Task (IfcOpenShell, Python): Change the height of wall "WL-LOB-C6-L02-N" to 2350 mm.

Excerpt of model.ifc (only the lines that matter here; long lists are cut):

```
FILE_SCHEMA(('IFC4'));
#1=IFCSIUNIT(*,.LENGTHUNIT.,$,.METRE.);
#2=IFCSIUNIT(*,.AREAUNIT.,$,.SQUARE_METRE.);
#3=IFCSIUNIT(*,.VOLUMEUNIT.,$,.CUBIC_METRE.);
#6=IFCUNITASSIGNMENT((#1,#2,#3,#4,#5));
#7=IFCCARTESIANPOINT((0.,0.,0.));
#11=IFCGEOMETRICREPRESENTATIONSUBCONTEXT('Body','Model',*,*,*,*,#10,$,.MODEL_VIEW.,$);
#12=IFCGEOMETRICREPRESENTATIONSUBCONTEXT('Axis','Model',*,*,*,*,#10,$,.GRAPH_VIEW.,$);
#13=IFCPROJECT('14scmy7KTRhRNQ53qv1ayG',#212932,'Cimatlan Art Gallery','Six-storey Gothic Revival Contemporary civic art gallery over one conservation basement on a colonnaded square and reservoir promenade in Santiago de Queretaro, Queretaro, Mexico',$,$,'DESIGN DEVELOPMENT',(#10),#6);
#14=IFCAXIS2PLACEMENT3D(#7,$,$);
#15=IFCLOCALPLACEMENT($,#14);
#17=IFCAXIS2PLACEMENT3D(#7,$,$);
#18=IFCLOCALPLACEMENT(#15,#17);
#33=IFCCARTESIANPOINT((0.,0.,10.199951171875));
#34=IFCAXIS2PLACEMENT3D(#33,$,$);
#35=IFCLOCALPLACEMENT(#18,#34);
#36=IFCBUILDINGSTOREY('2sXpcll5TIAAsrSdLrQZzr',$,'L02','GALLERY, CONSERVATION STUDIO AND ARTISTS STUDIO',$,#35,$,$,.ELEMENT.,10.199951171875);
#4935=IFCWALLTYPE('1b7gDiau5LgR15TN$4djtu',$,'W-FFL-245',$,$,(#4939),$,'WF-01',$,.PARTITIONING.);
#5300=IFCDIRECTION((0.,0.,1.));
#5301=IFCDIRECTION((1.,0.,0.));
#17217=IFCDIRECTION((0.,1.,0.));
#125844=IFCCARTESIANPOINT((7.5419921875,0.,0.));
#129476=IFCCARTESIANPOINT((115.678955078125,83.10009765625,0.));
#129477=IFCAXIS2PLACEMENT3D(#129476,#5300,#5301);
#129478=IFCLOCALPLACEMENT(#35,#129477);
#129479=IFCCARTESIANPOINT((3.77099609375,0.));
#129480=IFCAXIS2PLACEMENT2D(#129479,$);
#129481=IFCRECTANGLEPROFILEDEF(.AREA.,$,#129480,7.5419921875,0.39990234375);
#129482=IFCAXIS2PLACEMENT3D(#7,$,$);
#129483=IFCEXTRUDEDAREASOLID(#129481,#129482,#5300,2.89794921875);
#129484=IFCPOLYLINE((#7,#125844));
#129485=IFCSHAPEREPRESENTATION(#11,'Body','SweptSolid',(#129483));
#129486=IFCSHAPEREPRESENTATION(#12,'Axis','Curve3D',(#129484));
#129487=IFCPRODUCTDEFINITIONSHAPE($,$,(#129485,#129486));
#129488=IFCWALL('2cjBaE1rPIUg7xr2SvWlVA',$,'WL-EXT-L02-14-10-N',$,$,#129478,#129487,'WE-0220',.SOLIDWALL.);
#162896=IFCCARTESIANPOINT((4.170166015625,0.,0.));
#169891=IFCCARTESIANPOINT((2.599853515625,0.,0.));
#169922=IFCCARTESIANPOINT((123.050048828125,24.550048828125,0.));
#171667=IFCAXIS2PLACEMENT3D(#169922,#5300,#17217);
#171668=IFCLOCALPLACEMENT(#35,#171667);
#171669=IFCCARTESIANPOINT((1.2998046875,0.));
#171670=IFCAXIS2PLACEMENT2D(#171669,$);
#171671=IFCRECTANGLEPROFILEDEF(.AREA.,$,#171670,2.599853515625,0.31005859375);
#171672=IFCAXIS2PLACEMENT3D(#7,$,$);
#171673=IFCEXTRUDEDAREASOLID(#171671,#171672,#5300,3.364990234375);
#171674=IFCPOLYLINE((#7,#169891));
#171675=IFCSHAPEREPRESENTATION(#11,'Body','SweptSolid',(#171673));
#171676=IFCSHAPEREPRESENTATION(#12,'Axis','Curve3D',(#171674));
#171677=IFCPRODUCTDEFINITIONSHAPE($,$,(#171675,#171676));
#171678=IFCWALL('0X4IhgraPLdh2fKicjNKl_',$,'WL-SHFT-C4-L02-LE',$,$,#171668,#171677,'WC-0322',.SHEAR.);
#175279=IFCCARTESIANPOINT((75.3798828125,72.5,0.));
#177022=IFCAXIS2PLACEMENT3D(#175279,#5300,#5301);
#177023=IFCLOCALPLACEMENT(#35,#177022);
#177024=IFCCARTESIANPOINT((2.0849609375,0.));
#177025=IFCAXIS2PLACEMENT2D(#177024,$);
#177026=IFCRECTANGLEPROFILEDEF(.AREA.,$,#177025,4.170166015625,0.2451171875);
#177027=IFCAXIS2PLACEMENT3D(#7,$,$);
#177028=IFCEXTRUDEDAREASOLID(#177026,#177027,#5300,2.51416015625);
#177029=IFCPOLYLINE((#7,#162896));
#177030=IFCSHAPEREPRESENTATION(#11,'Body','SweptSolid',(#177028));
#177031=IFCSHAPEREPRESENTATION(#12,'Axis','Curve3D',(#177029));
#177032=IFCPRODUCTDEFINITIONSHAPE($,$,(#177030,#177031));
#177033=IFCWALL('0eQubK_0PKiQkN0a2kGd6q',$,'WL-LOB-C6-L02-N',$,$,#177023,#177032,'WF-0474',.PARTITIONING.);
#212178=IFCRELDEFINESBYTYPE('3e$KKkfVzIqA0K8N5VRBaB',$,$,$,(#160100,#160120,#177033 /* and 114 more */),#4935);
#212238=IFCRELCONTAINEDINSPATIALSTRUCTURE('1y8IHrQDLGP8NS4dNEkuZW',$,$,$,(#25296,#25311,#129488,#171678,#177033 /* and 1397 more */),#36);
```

```python
import ifcopenshell
import ifcopenshell.geom
import ifcopenshell.util.representation
import ifcopenshell.util.shape
import ifcopenshell.util.unit

model = ifcopenshell.open("model.ifc")
unit_scale = ifcopenshell.util.unit.calculate_unit_scale(model)
settings = ifcopenshell.geom.settings()


def volume(element):
    """Net volume in cubic metres, openings subtracted."""
    shape = ifcopenshell.geom.create_shape(settings, element)
    return ifcopenshell.util.shape.get_volume(shape.geometry)


wall = model.by_guid("0eQubK_0PKiQkN0a2kGd6q")
before = volume(wall)

body = ifcopenshell.util.representation.get_representation(wall, "Model", "Body")
solid = body.Items[0]
old_height = solid.Depth
solid.Depth = 2.35 / unit_scale
after = volume(wall)

print(f"height {old_height:g} -> {solid.Depth:g}, volume {before:.3f} -> {after:.3f} m3")

model.write("model_rev.ifc")
```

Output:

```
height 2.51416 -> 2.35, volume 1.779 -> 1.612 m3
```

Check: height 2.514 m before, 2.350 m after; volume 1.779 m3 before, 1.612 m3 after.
